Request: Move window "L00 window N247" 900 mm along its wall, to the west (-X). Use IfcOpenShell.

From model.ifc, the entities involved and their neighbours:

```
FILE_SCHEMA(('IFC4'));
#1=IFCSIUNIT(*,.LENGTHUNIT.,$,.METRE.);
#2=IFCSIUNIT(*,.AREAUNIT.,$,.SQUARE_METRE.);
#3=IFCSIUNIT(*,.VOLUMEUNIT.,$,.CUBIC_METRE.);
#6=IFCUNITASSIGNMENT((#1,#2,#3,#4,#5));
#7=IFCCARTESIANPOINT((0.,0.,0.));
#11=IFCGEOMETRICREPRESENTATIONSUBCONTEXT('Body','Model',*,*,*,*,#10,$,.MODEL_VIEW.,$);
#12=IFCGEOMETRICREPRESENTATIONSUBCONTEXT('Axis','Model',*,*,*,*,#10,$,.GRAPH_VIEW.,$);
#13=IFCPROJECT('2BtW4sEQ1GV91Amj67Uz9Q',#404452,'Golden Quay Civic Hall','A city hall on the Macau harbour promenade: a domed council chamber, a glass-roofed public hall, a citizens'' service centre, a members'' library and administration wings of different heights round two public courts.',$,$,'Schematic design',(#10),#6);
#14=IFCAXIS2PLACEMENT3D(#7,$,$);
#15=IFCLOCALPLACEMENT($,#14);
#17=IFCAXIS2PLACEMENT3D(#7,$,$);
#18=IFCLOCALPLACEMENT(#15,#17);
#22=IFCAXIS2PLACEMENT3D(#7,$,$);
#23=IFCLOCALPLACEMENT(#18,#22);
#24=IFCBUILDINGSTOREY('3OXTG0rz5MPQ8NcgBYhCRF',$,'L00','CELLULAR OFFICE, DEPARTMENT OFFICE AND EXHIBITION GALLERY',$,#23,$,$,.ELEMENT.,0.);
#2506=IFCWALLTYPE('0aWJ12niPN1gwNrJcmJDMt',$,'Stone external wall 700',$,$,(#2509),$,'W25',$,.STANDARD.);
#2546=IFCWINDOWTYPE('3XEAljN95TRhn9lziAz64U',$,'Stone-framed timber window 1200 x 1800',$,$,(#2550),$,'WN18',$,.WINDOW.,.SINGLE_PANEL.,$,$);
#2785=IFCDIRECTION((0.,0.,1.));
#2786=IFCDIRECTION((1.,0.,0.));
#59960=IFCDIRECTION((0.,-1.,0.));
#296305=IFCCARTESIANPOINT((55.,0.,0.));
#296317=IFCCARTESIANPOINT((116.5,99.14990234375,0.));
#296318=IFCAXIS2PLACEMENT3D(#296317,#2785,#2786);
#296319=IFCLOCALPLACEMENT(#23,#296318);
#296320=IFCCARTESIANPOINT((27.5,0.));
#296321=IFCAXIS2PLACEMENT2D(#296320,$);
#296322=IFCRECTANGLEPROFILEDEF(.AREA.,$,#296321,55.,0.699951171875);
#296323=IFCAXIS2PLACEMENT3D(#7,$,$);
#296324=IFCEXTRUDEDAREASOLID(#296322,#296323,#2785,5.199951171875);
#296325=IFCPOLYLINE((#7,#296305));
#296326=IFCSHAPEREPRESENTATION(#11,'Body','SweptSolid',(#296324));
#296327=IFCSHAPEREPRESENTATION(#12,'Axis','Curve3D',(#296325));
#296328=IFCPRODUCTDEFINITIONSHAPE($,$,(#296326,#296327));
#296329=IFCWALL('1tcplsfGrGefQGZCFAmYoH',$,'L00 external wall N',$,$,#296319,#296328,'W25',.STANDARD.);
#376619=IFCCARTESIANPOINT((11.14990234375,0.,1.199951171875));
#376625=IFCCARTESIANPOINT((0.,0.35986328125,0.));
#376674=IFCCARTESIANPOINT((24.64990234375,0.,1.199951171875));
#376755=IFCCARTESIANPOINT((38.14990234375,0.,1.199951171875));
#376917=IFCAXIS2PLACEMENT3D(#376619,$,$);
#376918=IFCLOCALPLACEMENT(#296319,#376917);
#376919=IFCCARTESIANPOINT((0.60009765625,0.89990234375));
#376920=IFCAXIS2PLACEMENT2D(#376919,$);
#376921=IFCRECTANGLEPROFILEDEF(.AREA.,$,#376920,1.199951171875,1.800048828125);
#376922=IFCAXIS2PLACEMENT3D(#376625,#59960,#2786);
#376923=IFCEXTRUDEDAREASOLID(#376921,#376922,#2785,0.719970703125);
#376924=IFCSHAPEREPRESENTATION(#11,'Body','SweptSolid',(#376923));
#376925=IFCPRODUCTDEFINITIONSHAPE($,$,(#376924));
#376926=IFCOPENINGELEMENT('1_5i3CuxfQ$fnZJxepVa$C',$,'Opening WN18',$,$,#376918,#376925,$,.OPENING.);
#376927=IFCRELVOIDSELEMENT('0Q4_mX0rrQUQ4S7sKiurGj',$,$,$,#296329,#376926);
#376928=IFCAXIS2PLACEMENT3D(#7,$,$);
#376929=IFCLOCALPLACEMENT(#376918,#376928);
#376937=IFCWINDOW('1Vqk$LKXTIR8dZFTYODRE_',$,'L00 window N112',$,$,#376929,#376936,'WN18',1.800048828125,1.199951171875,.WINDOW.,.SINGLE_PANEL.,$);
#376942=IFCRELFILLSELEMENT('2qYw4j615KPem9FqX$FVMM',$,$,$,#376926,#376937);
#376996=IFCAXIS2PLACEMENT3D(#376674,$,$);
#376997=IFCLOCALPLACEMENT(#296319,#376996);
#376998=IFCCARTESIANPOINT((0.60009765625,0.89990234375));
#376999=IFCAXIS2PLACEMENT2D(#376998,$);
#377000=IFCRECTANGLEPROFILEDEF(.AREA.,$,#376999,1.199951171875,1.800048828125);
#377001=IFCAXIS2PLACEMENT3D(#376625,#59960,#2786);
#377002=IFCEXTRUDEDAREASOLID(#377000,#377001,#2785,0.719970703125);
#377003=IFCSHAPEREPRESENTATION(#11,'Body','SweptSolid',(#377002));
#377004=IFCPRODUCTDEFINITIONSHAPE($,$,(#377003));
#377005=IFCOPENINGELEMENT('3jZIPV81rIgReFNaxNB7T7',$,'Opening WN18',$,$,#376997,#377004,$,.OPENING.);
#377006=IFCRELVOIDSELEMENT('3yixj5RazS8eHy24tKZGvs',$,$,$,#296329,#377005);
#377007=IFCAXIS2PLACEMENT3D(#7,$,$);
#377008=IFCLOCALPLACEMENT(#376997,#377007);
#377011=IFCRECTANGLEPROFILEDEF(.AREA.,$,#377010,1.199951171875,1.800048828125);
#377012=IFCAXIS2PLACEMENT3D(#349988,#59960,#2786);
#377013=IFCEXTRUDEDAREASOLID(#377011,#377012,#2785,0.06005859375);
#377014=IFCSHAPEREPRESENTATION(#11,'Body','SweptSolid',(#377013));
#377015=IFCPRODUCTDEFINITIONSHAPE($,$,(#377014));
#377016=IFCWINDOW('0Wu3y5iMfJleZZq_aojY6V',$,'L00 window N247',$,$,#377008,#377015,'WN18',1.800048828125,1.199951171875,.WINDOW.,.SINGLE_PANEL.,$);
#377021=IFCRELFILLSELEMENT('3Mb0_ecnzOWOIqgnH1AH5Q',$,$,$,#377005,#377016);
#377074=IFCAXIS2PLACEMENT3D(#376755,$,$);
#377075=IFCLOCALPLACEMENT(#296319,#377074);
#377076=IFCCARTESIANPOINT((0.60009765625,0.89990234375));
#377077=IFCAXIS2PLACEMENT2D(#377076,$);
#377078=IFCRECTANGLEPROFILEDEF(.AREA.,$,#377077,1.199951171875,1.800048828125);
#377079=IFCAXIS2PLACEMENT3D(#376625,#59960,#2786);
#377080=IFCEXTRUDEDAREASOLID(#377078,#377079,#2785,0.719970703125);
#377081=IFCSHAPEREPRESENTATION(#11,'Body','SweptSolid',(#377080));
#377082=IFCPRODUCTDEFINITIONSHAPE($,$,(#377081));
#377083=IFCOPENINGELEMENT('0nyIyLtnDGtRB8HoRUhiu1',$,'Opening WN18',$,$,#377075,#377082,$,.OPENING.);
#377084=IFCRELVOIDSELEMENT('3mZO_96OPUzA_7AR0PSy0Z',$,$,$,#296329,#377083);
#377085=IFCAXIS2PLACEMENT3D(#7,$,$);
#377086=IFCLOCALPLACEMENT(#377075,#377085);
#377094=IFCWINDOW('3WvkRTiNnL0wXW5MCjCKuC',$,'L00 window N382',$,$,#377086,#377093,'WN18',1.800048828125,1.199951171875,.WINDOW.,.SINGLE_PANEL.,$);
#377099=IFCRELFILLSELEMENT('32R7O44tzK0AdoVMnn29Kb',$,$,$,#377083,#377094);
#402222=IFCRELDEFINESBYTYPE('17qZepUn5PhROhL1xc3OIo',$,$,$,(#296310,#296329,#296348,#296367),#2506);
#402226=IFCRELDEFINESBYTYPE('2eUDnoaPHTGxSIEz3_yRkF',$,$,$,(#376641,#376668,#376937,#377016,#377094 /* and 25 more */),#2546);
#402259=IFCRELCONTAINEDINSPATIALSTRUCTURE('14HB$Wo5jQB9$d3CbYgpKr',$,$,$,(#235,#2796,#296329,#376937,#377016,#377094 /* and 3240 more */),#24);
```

```python
import ifcopenshell
import ifcopenshell.api.geometry
import ifcopenshell.util.placement
import ifcopenshell.util.unit

model = ifcopenshell.open("model.ifc")
unit_scale = ifcopenshell.util.unit.calculate_unit_scale(model)

window = model.by_guid("0Wu3y5iMfJleZZq_aojY6V")
opening = window.FillsVoids[0].RelatingOpeningElement
wall = opening.VoidsElements[0].RelatingBuildingElement

wall_matrix = ifcopenshell.util.placement.get_local_placement(wall.ObjectPlacement)
shift = wall_matrix[:3, 0] * -0.9 / unit_scale
before = ifcopenshell.util.placement.get_local_placement(window.ObjectPlacement)[:3, 3].copy()

# The window is placed relative to its opening, so it follows when the opening moves.
matrix = ifcopenshell.util.placement.get_local_placement(opening.ObjectPlacement)
matrix[:3, 3] += shift
ifcopenshell.api.geometry.edit_object_placement(
    model, product=opening, matrix=matrix, is_si=False, should_transform_children=True
)

after = ifcopenshell.util.placement.get_local_placement(window.ObjectPlacement)[:3, 3]
print("window moved by", (after - before).round(3) + 0.0)

model.write("model-out.ifc")
```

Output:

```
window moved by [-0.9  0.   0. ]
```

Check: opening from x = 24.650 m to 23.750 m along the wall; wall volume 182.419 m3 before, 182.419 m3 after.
